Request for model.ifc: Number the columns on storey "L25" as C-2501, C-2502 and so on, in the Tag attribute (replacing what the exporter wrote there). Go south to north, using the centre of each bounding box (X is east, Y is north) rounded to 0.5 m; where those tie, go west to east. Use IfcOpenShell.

First a look at what the model holds.

```python
import ifcopenshell
import ifcopenshell.util.element
import ifcopenshell.util.placement

model = ifcopenshell.open("model.ifc")
print(model.schema)
storey = next(s for s in model.by_type("IfcBuildingStorey") if s.Name == "L25")
columns = [e for e in ifcopenshell.util.element.get_decomposition(storey) if e.is_a("IfcColumn")]
for e in sorted(columns, key=lambda e: e.id()):
    origin = ifcopenshell.util.placement.get_local_placement(e.ObjectPlacement)[:3, 3]
    print(e.id(), e.Tag, e.Name, origin.round(2) + 0.0, sep=" | ")
```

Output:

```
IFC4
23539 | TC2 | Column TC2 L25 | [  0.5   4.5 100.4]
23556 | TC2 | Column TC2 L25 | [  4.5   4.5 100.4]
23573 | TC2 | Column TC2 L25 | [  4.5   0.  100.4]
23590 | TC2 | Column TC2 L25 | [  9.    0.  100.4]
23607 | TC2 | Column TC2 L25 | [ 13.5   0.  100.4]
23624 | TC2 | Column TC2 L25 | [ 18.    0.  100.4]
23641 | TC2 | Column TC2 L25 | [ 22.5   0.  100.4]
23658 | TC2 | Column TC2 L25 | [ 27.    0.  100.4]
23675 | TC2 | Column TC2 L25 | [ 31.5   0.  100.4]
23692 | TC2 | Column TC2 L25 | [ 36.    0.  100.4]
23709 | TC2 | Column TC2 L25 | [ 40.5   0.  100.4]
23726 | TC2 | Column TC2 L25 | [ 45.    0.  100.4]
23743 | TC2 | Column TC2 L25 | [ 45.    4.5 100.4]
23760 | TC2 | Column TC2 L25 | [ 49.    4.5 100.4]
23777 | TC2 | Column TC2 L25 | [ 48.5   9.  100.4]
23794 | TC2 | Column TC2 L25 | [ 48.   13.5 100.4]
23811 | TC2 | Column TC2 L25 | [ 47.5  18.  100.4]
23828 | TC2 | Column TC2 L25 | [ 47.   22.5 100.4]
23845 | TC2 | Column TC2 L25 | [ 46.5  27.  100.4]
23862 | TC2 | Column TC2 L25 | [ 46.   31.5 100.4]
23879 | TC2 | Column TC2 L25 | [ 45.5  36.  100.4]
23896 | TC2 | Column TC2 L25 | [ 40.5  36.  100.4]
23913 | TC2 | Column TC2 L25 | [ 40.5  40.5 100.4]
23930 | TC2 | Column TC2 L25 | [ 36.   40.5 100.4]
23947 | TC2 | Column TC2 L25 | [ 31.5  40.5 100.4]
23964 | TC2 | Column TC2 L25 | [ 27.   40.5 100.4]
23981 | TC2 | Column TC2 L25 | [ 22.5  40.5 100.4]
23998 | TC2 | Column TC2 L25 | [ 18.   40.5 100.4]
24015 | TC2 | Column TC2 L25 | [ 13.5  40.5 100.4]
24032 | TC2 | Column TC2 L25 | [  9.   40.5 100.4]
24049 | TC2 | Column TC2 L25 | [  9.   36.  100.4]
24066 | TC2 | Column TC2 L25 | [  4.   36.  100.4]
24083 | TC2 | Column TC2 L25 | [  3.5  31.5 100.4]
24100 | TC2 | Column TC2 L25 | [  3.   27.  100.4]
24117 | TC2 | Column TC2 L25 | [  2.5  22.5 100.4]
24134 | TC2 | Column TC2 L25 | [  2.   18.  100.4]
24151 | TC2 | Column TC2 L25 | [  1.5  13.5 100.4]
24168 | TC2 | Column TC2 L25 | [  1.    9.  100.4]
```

```python
import ifcopenshell
import ifcopenshell.geom
import ifcopenshell.util.element
import ifcopenshell.util.shape

model = ifcopenshell.open("model.ifc")
settings = ifcopenshell.geom.settings()
settings.set("use-world-coords", True)


def centre(element):
    shape = ifcopenshell.geom.create_shape(settings, element)
    return ifcopenshell.util.shape.get_bbox_centroid(shape.geometry)


storey = next(s for s in model.by_type("IfcBuildingStorey") if s.Name == "L25")
columns = [e for e in ifcopenshell.util.element.get_decomposition(storey) if e.is_a("IfcColumn")]

# Insertion points can sit at a corner or the storey origin, so sort by the geometry (in metres).
centres = {e: centre(e) for e in columns}
columns.sort(key=lambda e: (round(centres[e][1] / 0.5), centres[e][0]))

for i, e in enumerate(columns, start=1):
    number = f"C-25{i:02d}"
    e.Tag = number
    print(e.id(), number)

model.write("model_edited.ifc")
```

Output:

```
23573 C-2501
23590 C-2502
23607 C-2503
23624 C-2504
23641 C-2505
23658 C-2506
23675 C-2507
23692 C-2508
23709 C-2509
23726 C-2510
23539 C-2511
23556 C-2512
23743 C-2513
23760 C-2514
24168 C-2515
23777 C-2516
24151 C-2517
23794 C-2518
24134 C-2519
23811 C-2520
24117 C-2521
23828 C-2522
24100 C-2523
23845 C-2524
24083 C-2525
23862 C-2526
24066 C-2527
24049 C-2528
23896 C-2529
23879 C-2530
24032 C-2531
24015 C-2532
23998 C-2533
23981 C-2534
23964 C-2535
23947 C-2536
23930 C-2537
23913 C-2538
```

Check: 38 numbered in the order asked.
